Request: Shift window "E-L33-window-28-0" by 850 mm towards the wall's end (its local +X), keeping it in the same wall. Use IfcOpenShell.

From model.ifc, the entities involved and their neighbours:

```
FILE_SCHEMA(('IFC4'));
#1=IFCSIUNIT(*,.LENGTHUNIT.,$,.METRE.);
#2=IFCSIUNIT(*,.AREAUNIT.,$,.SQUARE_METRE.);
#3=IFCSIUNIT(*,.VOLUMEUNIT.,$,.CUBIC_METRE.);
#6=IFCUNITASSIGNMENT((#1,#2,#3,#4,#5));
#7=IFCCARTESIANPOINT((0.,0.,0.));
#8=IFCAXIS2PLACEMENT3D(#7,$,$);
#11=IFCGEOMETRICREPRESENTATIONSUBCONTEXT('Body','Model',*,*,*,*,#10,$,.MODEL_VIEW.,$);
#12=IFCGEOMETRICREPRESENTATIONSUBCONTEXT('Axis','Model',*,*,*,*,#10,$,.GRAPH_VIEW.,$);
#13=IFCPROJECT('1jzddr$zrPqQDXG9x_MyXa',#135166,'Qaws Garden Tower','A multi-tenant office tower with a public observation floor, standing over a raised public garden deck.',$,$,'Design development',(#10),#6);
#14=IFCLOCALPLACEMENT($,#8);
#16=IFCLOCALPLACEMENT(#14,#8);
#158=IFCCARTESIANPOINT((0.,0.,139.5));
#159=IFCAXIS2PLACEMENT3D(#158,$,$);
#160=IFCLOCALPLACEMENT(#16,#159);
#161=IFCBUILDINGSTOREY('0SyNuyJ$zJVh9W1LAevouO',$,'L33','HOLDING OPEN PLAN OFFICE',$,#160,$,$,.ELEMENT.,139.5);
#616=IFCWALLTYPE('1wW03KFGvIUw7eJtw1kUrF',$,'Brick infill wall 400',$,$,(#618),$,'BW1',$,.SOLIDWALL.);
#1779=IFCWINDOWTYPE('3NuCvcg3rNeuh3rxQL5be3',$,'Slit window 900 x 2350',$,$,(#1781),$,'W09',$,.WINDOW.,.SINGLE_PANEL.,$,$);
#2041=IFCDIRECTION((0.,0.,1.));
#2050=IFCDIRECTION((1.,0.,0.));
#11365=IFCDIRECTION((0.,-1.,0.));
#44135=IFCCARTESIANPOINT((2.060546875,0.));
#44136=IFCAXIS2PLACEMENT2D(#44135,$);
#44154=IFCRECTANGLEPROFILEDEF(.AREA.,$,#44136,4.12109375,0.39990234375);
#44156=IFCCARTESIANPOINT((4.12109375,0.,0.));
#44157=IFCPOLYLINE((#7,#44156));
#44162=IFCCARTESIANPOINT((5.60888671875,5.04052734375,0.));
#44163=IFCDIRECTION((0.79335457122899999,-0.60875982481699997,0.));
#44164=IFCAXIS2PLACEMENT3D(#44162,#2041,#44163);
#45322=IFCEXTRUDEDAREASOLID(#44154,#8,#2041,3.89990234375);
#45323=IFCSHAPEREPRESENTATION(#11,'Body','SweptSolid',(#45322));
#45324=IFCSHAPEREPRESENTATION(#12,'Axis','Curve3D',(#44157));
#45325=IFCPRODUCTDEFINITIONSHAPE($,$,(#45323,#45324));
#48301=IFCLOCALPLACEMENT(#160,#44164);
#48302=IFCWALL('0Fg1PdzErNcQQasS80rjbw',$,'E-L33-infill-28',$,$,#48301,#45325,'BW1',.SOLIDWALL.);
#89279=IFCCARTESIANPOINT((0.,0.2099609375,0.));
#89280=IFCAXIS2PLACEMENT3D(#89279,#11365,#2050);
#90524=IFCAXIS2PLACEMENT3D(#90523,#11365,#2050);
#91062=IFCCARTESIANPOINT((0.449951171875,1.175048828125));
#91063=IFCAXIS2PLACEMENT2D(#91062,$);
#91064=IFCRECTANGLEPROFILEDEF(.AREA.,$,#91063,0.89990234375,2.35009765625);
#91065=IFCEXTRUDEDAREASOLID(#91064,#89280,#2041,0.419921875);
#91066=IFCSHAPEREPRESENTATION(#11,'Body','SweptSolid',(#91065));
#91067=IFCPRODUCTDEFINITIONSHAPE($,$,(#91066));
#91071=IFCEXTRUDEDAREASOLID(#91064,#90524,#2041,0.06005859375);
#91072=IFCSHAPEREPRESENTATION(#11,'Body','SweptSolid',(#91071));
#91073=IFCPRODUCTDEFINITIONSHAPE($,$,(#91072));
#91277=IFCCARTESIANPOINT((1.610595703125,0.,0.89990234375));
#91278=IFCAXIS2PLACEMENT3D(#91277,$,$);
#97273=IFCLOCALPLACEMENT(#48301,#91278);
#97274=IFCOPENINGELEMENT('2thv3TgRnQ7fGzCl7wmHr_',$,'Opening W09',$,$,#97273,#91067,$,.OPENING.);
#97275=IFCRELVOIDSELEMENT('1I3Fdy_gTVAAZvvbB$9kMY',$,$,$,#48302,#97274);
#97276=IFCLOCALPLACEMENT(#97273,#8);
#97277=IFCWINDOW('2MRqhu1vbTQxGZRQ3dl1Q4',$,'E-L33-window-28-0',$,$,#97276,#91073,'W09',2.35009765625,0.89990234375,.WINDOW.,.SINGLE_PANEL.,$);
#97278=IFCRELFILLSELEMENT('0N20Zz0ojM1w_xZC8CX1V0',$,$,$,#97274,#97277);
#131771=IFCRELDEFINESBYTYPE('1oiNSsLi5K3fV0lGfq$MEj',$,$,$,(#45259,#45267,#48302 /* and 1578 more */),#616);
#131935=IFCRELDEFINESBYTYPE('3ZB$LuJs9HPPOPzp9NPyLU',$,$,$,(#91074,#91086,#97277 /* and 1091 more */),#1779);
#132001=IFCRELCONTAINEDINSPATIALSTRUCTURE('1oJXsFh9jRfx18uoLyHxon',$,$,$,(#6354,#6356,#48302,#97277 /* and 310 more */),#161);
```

```python
import ifcopenshell
import ifcopenshell.api.geometry
import ifcopenshell.util.placement

model = ifcopenshell.open("model.ifc")

window = model.by_guid("2MRqhu1vbTQxGZRQ3dl1Q4")
opening = window.FillsVoids[0].RelatingOpeningElement
wall = opening.VoidsElements[0].RelatingBuildingElement

wall_matrix = ifcopenshell.util.placement.get_local_placement(wall.ObjectPlacement)
shift = wall_matrix[:3, 0] * 0.85
before = ifcopenshell.util.placement.get_local_placement(window.ObjectPlacement)[:3, 3].copy()

# The window is placed relative to its opening, so it follows when the opening moves.
matrix = ifcopenshell.util.placement.get_local_placement(opening.ObjectPlacement)
matrix[:3, 3] += shift
ifcopenshell.api.geometry.edit_object_placement(
    model, product=opening, matrix=matrix, is_si=False, should_transform_children=True
)

after = ifcopenshell.util.placement.get_local_placement(window.ObjectPlacement)[:3, 3]
print("window moved by", (after - before).round(3) + 0.0)

model.write("model_updated.ifc")
```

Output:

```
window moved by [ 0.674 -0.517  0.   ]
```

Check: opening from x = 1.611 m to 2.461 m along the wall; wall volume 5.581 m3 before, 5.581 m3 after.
